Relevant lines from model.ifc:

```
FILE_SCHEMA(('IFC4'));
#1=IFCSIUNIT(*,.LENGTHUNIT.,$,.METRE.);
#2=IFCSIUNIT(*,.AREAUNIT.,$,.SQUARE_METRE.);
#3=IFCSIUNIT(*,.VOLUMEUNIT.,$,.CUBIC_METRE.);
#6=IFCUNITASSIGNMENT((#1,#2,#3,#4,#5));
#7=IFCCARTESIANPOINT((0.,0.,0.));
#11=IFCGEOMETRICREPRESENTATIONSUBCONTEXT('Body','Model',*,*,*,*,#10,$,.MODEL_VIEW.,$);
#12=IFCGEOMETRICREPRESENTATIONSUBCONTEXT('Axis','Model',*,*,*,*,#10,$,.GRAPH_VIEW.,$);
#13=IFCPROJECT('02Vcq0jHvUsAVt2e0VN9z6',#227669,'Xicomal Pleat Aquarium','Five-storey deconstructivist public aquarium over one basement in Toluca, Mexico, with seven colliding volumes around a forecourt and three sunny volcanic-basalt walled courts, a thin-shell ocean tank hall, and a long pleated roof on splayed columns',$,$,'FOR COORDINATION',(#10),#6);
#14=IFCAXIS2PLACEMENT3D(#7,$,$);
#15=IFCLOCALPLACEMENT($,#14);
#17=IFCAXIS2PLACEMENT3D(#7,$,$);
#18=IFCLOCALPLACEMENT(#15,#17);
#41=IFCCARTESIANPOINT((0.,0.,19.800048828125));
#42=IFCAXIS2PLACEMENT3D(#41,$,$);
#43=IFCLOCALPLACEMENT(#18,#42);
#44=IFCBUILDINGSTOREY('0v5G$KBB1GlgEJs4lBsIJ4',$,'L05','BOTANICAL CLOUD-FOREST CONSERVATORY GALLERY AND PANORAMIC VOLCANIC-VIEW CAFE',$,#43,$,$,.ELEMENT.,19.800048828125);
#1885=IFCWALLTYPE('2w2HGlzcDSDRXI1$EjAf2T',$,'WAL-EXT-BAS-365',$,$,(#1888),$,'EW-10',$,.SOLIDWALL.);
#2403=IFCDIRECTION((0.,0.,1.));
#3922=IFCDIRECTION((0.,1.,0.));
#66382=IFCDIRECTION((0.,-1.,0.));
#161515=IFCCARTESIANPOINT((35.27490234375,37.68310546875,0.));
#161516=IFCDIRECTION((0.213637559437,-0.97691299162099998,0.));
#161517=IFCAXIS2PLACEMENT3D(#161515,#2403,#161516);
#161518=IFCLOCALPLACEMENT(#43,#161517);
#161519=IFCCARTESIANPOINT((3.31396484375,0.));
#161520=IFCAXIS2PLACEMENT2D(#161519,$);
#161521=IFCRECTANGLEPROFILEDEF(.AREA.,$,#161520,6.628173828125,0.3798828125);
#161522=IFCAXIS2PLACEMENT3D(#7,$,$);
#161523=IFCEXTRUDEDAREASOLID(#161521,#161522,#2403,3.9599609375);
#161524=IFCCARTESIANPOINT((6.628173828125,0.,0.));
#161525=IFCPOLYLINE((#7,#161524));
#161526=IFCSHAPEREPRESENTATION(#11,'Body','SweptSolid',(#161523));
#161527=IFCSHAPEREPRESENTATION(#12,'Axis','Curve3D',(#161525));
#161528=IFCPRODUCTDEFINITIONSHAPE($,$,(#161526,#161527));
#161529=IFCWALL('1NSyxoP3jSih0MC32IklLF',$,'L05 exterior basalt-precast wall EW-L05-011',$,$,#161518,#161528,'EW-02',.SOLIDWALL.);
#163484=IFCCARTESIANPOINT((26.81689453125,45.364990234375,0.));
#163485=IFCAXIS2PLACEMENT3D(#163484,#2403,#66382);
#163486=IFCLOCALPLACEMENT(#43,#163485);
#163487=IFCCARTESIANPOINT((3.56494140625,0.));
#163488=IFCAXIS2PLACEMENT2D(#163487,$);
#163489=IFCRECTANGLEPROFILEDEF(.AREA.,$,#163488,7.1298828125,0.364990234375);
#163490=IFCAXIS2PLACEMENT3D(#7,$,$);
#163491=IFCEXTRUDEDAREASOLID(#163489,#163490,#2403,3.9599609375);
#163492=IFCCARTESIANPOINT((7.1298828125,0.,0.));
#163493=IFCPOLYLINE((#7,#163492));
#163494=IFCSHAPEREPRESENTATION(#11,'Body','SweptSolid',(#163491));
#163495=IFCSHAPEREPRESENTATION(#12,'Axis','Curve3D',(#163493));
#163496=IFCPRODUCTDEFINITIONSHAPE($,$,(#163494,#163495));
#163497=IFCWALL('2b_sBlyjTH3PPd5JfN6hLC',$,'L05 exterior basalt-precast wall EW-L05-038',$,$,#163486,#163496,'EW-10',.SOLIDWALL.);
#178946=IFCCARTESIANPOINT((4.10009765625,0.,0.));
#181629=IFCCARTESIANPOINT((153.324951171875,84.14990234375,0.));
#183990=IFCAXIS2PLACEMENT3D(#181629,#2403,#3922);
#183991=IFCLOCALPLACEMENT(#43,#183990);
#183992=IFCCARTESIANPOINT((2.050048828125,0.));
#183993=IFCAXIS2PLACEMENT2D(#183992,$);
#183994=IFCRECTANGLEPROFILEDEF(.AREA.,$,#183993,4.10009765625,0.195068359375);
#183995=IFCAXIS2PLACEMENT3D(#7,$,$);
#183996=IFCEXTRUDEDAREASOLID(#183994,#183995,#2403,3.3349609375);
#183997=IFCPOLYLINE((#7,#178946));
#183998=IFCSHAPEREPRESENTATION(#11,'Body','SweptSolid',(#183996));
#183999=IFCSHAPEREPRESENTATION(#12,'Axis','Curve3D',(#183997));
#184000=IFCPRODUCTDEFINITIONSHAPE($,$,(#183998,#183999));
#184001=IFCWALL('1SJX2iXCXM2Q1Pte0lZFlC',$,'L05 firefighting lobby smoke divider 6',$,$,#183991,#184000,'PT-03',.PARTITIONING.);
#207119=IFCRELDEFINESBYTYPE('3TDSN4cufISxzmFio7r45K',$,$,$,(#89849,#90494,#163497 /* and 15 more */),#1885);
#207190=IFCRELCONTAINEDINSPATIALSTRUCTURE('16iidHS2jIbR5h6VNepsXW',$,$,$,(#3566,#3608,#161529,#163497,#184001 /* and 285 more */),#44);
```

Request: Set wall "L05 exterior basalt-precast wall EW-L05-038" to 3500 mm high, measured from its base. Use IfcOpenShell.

```python
import ifcopenshell
import ifcopenshell.geom
import ifcopenshell.util.representation
import ifcopenshell.util.shape
import ifcopenshell.util.unit

model = ifcopenshell.open("model.ifc")
unit_scale = ifcopenshell.util.unit.calculate_unit_scale(model)
settings = ifcopenshell.geom.settings()


def volume(element):
    """Net volume in cubic metres, openings subtracted."""
    shape = ifcopenshell.geom.create_shape(settings, element)
    return ifcopenshell.util.shape.get_volume(shape.geometry)


wall = model.by_guid("2b_sBlyjTH3PPd5JfN6hLC")
before = volume(wall)

body = ifcopenshell.util.representation.get_representation(wall, "Model", "Body")
solid = body.Items[0]
old_height = solid.Depth
solid.Depth = 3.5 / unit_scale
after = volume(wall)

print(f"height {old_height:g} -> {solid.Depth:g}, volume {before:.3f} -> {after:.3f} m3")

model.write("model_rev.ifc")
```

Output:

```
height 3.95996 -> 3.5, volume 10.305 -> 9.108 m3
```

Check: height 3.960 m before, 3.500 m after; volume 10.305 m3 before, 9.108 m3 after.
